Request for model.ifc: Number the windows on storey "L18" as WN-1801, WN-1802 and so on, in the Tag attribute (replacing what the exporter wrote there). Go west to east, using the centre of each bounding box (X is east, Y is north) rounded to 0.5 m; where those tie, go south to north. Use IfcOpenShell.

First a look at what the model holds.

```python
import ifcopenshell
import ifcopenshell.util.element
import ifcopenshell.util.placement

model = ifcopenshell.open("model.ifc")
print(model.schema)
storey = next(s for s in model.by_type("IfcBuildingStorey") if s.Name == "L18")
windows = [e for e in ifcopenshell.util.element.get_decomposition(storey) if e.is_a("IfcWindow")]
for e in sorted(windows, key=lambda e: e.id()):
    origin = ifcopenshell.util.placement.get_local_placement(e.ObjectPlacement)[:3, 3]
    print(e.id(), e.Tag, e.Name, origin.round(2) + 0.0, sep=" | ")
```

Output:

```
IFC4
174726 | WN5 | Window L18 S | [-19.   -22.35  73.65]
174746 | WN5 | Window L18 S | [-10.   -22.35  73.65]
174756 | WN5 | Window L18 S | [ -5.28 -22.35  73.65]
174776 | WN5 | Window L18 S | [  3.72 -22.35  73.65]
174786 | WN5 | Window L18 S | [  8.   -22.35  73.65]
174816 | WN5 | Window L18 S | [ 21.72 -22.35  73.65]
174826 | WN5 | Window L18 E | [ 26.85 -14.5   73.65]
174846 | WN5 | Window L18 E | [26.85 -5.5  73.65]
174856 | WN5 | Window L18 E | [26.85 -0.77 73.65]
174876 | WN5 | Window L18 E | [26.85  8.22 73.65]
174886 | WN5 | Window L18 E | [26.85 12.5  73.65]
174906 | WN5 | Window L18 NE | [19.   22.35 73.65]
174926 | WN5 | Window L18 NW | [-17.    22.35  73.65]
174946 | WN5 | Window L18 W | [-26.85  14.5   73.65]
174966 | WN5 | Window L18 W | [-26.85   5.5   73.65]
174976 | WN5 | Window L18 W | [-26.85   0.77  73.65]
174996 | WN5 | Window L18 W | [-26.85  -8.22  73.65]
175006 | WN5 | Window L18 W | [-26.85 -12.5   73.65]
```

```python
import ifcopenshell
import ifcopenshell.geom
import ifcopenshell.util.element
import ifcopenshell.util.shape

model = ifcopenshell.open("model.ifc")
settings = ifcopenshell.geom.settings()
settings.set("use-world-coords", True)


def centre(element):
    shape = ifcopenshell.geom.create_shape(settings, element)
    return ifcopenshell.util.shape.get_bbox_centroid(shape.geometry)


storey = next(s for s in model.by_type("IfcBuildingStorey") if s.Name == "L18")
windows = [e for e in ifcopenshell.util.element.get_decomposition(storey) if e.is_a("IfcWindow")]

# Insertion points can sit at a corner or the storey origin, so sort by the geometry (in metres).
centres = {e: centre(e) for e in windows}
windows.sort(key=lambda e: (round(centres[e][0] / 0.5), centres[e][1]))

for i, e in enumerate(windows, start=1):
    number = f"WN-18{i:02d}"
    e.Tag = number
    print(e.id(), number)

model.write("model_updated.ifc")
```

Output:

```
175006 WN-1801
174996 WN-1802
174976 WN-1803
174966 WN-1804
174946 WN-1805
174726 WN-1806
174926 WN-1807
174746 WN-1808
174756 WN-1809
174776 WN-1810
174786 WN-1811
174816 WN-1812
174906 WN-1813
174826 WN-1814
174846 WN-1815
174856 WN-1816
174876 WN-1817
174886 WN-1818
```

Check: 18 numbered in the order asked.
